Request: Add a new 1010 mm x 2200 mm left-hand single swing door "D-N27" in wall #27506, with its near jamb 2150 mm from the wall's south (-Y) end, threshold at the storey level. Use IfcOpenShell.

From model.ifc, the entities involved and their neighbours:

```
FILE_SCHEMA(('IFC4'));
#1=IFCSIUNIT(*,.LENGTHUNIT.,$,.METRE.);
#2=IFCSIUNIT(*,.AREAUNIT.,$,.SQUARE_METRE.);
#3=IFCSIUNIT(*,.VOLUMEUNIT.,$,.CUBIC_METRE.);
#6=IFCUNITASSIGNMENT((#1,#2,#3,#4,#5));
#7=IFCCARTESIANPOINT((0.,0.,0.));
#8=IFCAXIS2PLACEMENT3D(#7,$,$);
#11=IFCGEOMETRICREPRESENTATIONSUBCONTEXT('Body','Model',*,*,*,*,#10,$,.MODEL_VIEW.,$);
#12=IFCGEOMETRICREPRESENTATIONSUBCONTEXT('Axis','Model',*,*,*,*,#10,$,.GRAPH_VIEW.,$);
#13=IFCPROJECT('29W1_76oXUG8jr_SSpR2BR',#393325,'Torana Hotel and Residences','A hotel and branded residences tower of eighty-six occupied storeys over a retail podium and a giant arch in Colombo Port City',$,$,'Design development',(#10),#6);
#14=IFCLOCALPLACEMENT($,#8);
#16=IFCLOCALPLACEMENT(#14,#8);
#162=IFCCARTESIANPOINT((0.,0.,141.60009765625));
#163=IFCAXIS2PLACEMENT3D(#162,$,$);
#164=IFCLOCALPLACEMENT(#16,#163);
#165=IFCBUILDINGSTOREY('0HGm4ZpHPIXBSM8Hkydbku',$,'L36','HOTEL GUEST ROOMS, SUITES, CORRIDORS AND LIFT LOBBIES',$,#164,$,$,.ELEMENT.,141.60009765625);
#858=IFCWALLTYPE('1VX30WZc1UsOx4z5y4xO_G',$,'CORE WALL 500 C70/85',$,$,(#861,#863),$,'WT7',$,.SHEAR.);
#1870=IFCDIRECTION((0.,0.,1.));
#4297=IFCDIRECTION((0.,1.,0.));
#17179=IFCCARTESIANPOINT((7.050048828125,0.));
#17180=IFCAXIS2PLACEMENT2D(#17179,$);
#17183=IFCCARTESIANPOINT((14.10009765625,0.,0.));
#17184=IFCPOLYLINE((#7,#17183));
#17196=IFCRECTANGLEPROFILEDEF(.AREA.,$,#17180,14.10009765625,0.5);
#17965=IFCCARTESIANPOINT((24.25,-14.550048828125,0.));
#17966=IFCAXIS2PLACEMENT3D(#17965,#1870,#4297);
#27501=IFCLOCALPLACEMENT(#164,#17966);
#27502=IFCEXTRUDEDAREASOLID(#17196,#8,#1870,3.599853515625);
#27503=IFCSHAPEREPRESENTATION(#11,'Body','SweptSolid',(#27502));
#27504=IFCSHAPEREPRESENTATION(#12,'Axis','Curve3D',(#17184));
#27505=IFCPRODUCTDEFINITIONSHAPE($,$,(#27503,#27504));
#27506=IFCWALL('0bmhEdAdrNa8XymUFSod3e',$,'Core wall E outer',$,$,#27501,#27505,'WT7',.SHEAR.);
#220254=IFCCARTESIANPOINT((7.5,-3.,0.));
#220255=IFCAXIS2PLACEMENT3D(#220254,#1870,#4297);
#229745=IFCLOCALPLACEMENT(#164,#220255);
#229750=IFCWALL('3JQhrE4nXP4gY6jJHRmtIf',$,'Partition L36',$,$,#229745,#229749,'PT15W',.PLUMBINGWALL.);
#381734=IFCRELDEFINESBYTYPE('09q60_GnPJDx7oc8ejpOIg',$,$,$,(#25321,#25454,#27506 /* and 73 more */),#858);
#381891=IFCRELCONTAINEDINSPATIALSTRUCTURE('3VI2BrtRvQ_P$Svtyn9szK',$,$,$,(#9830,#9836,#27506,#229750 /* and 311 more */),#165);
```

```python
import numpy as np
import ifcopenshell
import ifcopenshell.api.feature
import ifcopenshell.api.geometry
import ifcopenshell.api.root
import ifcopenshell.api.spatial
import ifcopenshell.geom
import ifcopenshell.util.element
import ifcopenshell.util.placement
import ifcopenshell.util.representation
import ifcopenshell.util.shape
import ifcopenshell.util.unit

model = ifcopenshell.open("model.ifc")
unit_scale = ifcopenshell.util.unit.calculate_unit_scale(model)
settings = ifcopenshell.geom.settings()


def volume(element):
    """Net volume in cubic metres, openings subtracted."""
    shape = ifcopenshell.geom.create_shape(settings, element)
    return ifcopenshell.util.shape.get_volume(shape.geometry)


wall = model.by_guid("0bmhEdAdrNa8XymUFSod3e")
storey = ifcopenshell.util.element.get_container(wall, ifc_class="IfcBuildingStorey")
context = ifcopenshell.util.representation.get_context(model, "Model", "Body", "MODEL_VIEW")
before = volume(wall)

width, height, from_end, sill = 1.01, 2.2, 2.15, 0.0  # metres

# The wall runs along its own X axis, and the end named is its -X end.
wall_shape = ifcopenshell.geom.create_shape(settings, wall)
x, y, z = ifcopenshell.util.shape.get_vertices(wall_shape.geometry).T
start = x.min() + from_end
face, thickness = float(y.min()), float(y.max() - y.min())
wall_matrix = ifcopenshell.util.placement.get_local_placement(wall.ObjectPlacement)
level = ifcopenshell.util.placement.get_local_placement(storey.ObjectPlacement)[2, 3]


def in_wall(x, y):
    """Placement at x, y metres in the wall's axes, at sill height."""
    matrix = wall_matrix.copy()
    matrix[:, 3] = wall_matrix @ np.array([x / unit_scale, y / unit_scale, 0.0, 1.0])
    matrix[2, 3] = level + sill / unit_scale
    return matrix


# Opening: a box that overshoots both wall faces by 50 mm.
opening = ifcopenshell.api.root.create_entity(model, ifc_class="IfcOpeningElement", predefined_type="OPENING")
box = ifcopenshell.api.geometry.add_wall_representation(
    model, context=context, length=width, height=height, thickness=thickness + 0.1
)
ifcopenshell.api.geometry.assign_representation(model, product=opening, representation=box)
ifcopenshell.api.geometry.edit_object_placement(model, product=opening, matrix=in_wall(start, face - 0.05), is_si=False)
ifcopenshell.api.feature.add_feature(model, feature=opening, element=wall)

door = ifcopenshell.api.root.create_entity(model, ifc_class="IfcDoor", name="D-N27", predefined_type="DOOR")
door.OverallWidth, door.OverallHeight = width / unit_scale, height / unit_scale
door.OperationType = "SINGLE_SWING_LEFT"
body = ifcopenshell.api.geometry.add_door_representation(
    model,
    context=context,
    overall_width=door.OverallWidth,
    overall_height=door.OverallHeight,
    operation_type="SINGLE_SWING_LEFT",
    lining_properties={"LiningDepth": thickness / unit_scale, "ThresholdDepth": thickness / unit_scale},
)
ifcopenshell.api.geometry.assign_representation(model, product=door, representation=body)
ifcopenshell.api.spatial.assign_container(model, products=[door], relating_structure=storey)
ifcopenshell.api.feature.add_filling(model, opening=opening, element=door)

# The lining spans the wall, so the door starts at the wall face.
ifcopenshell.api.geometry.edit_object_placement(model, product=door, matrix=in_wall(start, face), is_si=False)

after = volume(wall)

print(f"wall volume {before:.3f} -> {after:.3f} m3")

model.write("model_v2.ifc")
```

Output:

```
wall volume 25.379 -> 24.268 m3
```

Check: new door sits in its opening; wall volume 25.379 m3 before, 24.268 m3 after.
